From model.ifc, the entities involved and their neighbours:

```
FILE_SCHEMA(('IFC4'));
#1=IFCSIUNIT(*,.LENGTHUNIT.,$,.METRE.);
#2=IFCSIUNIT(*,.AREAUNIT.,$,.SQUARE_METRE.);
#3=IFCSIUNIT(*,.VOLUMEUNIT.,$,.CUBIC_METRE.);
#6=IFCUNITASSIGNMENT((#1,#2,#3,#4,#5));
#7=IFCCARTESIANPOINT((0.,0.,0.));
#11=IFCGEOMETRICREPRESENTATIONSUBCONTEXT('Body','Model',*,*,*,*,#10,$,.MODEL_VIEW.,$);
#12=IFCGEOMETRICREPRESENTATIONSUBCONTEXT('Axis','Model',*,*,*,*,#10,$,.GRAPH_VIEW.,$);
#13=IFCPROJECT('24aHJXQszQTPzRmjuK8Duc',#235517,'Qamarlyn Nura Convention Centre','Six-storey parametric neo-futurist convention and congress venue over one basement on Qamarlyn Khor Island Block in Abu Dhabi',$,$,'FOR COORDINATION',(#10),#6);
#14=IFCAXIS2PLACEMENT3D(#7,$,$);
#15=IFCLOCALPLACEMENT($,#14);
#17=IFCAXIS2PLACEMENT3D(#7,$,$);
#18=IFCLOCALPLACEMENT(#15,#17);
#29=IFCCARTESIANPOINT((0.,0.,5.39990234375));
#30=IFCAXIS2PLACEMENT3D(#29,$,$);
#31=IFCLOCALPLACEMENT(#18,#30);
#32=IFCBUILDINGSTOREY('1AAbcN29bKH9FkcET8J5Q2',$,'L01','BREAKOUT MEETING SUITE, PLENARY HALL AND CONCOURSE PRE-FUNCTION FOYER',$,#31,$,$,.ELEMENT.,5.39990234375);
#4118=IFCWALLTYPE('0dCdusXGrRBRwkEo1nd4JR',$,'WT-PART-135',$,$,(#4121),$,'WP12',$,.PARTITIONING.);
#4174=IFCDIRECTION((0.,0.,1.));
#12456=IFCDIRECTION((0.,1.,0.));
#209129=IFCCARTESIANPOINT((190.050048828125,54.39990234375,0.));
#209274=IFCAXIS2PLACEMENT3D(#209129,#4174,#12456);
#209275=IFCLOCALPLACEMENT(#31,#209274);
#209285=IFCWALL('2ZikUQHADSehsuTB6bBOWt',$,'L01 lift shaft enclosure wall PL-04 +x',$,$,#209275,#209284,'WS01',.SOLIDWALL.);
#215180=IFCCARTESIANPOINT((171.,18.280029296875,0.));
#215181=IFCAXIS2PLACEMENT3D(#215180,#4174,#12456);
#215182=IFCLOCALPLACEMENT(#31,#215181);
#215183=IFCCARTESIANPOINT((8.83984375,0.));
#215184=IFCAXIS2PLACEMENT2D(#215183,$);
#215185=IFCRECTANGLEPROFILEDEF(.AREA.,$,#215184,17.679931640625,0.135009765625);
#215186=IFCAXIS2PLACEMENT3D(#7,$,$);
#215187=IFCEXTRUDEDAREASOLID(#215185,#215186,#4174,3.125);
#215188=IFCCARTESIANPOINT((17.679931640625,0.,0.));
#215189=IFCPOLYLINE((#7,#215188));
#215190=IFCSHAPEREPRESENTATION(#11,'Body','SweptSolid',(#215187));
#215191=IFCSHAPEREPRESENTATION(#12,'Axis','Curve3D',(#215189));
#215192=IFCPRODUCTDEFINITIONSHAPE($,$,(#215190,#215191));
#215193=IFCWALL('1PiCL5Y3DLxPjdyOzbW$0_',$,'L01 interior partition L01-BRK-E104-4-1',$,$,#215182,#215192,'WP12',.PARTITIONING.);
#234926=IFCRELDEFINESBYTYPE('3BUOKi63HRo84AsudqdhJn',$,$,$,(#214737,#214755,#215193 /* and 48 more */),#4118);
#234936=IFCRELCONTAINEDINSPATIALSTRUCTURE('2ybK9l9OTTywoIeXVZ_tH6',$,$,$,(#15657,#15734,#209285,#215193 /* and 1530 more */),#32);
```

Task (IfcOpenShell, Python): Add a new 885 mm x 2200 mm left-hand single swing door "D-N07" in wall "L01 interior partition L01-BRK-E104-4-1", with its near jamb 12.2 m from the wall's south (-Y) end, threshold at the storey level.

```python
import numpy as np
import ifcopenshell
import ifcopenshell.api.feature
import ifcopenshell.api.geometry
import ifcopenshell.api.root
import ifcopenshell.api.spatial
import ifcopenshell.geom
import ifcopenshell.util.element
import ifcopenshell.util.placement
import ifcopenshell.util.representation
import ifcopenshell.util.shape
import ifcopenshell.util.unit

model = ifcopenshell.open("model.ifc")
unit_scale = ifcopenshell.util.unit.calculate_unit_scale(model)
settings = ifcopenshell.geom.settings()


def volume(element):
    """Net volume in cubic metres, openings subtracted."""
    shape = ifcopenshell.geom.create_shape(settings, element)
    return ifcopenshell.util.shape.get_volume(shape.geometry)


wall = model.by_guid("1PiCL5Y3DLxPjdyOzbW$0_")
storey = ifcopenshell.util.element.get_container(wall, ifc_class="IfcBuildingStorey")
context = ifcopenshell.util.representation.get_context(model, "Model", "Body", "MODEL_VIEW")
before = volume(wall)

width, height, from_end, sill = 0.885, 2.2, 12.2, 0.0  # metres

# The wall runs along its own X axis, and the end named is its -X end.
wall_shape = ifcopenshell.geom.create_shape(settings, wall)
x, y, z = ifcopenshell.util.shape.get_vertices(wall_shape.geometry).T
start = x.min() + from_end
face, thickness = float(y.min()), float(y.max() - y.min())
wall_matrix = ifcopenshell.util.placement.get_local_placement(wall.ObjectPlacement)
level = ifcopenshell.util.placement.get_local_placement(storey.ObjectPlacement)[2, 3]


def in_wall(x, y):
    """Placement at x, y metres in the wall's axes, at sill height."""
    matrix = wall_matrix.copy()
    matrix[:, 3] = wall_matrix @ np.array([x / unit_scale, y / unit_scale, 0.0, 1.0])
    matrix[2, 3] = level + sill / unit_scale
    return matrix


# Opening: a box that overshoots both wall faces by 50 mm.
opening = ifcopenshell.api.root.create_entity(model, ifc_class="IfcOpeningElement", predefined_type="OPENING")
box = ifcopenshell.api.geometry.add_wall_representation(
    model, context=context, length=width, height=height, thickness=thickness + 0.1
)
ifcopenshell.api.geometry.assign_representation(model, product=opening, representation=box)
ifcopenshell.api.geometry.edit_object_placement(model, product=opening, matrix=in_wall(start, face - 0.05), is_si=False)
ifcopenshell.api.feature.add_feature(model, feature=opening, element=wall)

door = ifcopenshell.api.root.create_entity(model, ifc_class="IfcDoor", name="D-N07", predefined_type="DOOR")
door.OverallWidth, door.OverallHeight = width / unit_scale, height / unit_scale
door.OperationType = "SINGLE_SWING_LEFT"
body = ifcopenshell.api.geometry.add_door_representation(
    model,
    context=context,
    overall_width=door.OverallWidth,
    overall_height=door.OverallHeight,
    operation_type="SINGLE_SWING_LEFT",
    lining_properties={"LiningDepth": thickness / unit_scale, "ThresholdDepth": thickness / unit_scale},
)
ifcopenshell.api.geometry.assign_representation(model, product=door, representation=body)
ifcopenshell.api.spatial.assign_container(model, products=[door], relating_structure=storey)
ifcopenshell.api.feature.add_filling(model, opening=opening, element=door)

# The lining spans the wall, so the door starts at the wall face.
ifcopenshell.api.geometry.edit_object_placement(model, product=door, matrix=in_wall(start, face), is_si=False)

after = volume(wall)

print(f"wall volume {before:.3f} -> {after:.3f} m3")

model.write("model_edited.ifc")
```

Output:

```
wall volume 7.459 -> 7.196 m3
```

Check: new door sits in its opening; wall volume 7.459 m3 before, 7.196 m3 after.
